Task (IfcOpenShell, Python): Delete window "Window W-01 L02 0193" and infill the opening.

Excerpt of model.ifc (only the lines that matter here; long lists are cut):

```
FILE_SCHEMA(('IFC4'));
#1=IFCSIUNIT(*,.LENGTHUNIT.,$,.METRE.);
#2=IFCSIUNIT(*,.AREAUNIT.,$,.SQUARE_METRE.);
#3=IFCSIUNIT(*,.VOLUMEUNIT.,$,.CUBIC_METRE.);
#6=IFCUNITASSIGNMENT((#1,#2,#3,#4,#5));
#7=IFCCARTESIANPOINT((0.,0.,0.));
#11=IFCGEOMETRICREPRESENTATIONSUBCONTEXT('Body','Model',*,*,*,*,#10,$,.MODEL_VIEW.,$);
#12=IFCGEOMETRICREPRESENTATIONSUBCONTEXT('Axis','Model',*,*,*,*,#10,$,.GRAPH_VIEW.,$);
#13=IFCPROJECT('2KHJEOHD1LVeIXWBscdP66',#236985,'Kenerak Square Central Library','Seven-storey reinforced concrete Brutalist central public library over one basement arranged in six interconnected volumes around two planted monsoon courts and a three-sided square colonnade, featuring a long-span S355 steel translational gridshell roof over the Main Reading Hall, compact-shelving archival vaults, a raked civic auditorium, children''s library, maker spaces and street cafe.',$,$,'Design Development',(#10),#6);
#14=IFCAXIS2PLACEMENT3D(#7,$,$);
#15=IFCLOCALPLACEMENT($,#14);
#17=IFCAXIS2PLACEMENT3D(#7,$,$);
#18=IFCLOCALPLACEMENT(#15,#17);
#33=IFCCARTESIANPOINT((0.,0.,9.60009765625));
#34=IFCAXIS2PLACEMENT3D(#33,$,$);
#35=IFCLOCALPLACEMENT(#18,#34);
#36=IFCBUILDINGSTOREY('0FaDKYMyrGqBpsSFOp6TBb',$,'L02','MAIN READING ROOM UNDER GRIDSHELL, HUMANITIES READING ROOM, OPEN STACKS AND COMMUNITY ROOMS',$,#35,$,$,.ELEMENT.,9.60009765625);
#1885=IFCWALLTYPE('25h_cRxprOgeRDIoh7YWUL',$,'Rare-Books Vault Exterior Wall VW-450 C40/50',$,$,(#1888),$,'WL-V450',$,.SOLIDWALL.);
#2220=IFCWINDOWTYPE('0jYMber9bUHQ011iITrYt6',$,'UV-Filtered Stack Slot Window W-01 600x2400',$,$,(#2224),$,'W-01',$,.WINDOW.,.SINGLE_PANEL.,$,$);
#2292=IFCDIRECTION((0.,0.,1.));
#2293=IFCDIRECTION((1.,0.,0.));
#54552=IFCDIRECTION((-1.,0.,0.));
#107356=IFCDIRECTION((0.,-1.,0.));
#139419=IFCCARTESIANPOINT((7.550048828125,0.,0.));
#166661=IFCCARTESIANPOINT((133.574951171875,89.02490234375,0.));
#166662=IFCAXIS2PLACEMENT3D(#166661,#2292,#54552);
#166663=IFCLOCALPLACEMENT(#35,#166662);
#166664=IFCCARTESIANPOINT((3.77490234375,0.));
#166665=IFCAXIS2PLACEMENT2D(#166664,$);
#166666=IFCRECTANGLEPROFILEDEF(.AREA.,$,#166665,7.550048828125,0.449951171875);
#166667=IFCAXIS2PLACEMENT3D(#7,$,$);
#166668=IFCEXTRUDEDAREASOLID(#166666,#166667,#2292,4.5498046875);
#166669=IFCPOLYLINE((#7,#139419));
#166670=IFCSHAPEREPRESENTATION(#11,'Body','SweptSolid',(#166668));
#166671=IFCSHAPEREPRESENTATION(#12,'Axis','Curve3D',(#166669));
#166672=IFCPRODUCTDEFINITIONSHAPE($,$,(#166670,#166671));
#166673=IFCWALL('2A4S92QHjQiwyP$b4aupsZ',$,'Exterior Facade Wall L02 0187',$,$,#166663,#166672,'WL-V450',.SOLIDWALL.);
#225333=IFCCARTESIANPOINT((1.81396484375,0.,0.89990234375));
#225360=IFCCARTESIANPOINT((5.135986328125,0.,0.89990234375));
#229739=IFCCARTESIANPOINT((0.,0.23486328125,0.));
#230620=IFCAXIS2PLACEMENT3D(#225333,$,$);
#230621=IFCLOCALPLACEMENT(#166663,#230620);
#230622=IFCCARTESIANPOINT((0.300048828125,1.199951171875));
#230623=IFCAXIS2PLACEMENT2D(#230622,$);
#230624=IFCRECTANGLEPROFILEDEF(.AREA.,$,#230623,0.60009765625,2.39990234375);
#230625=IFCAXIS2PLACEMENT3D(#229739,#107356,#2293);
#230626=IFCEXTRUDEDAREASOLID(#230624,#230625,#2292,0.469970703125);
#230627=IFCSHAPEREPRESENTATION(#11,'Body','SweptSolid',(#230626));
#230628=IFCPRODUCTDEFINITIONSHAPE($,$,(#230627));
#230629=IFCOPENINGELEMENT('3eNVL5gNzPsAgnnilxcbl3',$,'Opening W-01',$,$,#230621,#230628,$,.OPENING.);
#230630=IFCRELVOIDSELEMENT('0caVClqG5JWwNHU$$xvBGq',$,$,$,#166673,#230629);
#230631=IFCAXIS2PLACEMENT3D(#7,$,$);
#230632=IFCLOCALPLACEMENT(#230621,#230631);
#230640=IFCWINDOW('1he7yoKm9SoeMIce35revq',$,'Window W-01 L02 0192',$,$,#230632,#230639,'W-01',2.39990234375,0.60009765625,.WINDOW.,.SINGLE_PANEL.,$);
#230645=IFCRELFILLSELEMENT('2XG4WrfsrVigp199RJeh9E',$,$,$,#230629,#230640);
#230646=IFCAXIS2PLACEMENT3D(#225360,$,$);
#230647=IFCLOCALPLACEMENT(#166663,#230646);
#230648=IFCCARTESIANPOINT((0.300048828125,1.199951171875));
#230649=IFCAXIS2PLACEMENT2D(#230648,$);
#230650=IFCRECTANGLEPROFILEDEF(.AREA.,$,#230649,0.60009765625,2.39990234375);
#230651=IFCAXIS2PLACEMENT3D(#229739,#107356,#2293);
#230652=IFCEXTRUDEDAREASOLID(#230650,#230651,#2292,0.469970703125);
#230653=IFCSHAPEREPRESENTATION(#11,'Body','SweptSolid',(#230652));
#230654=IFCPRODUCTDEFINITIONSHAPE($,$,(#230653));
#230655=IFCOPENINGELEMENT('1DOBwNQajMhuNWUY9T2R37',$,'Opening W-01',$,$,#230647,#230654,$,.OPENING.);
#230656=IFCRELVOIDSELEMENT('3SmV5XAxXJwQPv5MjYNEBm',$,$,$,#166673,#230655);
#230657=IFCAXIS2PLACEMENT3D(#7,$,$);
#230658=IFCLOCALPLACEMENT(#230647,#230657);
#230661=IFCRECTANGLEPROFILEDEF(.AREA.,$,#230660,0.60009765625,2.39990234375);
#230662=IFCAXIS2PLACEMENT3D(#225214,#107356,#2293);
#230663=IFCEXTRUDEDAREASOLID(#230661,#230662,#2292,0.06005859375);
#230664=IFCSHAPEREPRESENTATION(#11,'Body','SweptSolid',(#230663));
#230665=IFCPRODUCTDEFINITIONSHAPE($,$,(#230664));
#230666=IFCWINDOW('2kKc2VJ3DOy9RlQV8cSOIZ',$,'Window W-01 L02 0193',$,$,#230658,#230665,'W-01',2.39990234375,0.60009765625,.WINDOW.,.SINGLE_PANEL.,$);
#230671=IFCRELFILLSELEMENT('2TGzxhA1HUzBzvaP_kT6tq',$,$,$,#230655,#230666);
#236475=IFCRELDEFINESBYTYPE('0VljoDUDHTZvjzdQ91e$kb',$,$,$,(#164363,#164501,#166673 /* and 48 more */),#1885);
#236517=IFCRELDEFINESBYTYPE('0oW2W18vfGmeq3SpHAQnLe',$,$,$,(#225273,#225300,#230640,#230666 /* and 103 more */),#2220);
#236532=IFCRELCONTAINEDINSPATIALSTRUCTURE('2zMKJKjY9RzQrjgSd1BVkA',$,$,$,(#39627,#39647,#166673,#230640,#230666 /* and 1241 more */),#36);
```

```python
import ifcopenshell
import ifcopenshell.api.feature
import ifcopenshell.api.root
import ifcopenshell.geom
import ifcopenshell.util.shape

model = ifcopenshell.open("model.ifc")
settings = ifcopenshell.geom.settings()


def volume(element):
    """Net volume in cubic metres, openings subtracted."""
    shape = ifcopenshell.geom.create_shape(settings, element)
    return ifcopenshell.util.shape.get_volume(shape.geometry)


window = model.by_guid("2kKc2VJ3DOy9RlQV8cSOIZ")
opening = window.FillsVoids[0].RelatingOpeningElement
wall = opening.VoidsElements[0].RelatingBuildingElement
before = volume(wall)

ifcopenshell.api.root.remove_product(model, product=window)
ifcopenshell.api.feature.remove_feature(model, feature=opening)

after = volume(wall)

print(f"wall volume {before:.3f} -> {after:.3f} m3")

model.write("model-out.ifc")
```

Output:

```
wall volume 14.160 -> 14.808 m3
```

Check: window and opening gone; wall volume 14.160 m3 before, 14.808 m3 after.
